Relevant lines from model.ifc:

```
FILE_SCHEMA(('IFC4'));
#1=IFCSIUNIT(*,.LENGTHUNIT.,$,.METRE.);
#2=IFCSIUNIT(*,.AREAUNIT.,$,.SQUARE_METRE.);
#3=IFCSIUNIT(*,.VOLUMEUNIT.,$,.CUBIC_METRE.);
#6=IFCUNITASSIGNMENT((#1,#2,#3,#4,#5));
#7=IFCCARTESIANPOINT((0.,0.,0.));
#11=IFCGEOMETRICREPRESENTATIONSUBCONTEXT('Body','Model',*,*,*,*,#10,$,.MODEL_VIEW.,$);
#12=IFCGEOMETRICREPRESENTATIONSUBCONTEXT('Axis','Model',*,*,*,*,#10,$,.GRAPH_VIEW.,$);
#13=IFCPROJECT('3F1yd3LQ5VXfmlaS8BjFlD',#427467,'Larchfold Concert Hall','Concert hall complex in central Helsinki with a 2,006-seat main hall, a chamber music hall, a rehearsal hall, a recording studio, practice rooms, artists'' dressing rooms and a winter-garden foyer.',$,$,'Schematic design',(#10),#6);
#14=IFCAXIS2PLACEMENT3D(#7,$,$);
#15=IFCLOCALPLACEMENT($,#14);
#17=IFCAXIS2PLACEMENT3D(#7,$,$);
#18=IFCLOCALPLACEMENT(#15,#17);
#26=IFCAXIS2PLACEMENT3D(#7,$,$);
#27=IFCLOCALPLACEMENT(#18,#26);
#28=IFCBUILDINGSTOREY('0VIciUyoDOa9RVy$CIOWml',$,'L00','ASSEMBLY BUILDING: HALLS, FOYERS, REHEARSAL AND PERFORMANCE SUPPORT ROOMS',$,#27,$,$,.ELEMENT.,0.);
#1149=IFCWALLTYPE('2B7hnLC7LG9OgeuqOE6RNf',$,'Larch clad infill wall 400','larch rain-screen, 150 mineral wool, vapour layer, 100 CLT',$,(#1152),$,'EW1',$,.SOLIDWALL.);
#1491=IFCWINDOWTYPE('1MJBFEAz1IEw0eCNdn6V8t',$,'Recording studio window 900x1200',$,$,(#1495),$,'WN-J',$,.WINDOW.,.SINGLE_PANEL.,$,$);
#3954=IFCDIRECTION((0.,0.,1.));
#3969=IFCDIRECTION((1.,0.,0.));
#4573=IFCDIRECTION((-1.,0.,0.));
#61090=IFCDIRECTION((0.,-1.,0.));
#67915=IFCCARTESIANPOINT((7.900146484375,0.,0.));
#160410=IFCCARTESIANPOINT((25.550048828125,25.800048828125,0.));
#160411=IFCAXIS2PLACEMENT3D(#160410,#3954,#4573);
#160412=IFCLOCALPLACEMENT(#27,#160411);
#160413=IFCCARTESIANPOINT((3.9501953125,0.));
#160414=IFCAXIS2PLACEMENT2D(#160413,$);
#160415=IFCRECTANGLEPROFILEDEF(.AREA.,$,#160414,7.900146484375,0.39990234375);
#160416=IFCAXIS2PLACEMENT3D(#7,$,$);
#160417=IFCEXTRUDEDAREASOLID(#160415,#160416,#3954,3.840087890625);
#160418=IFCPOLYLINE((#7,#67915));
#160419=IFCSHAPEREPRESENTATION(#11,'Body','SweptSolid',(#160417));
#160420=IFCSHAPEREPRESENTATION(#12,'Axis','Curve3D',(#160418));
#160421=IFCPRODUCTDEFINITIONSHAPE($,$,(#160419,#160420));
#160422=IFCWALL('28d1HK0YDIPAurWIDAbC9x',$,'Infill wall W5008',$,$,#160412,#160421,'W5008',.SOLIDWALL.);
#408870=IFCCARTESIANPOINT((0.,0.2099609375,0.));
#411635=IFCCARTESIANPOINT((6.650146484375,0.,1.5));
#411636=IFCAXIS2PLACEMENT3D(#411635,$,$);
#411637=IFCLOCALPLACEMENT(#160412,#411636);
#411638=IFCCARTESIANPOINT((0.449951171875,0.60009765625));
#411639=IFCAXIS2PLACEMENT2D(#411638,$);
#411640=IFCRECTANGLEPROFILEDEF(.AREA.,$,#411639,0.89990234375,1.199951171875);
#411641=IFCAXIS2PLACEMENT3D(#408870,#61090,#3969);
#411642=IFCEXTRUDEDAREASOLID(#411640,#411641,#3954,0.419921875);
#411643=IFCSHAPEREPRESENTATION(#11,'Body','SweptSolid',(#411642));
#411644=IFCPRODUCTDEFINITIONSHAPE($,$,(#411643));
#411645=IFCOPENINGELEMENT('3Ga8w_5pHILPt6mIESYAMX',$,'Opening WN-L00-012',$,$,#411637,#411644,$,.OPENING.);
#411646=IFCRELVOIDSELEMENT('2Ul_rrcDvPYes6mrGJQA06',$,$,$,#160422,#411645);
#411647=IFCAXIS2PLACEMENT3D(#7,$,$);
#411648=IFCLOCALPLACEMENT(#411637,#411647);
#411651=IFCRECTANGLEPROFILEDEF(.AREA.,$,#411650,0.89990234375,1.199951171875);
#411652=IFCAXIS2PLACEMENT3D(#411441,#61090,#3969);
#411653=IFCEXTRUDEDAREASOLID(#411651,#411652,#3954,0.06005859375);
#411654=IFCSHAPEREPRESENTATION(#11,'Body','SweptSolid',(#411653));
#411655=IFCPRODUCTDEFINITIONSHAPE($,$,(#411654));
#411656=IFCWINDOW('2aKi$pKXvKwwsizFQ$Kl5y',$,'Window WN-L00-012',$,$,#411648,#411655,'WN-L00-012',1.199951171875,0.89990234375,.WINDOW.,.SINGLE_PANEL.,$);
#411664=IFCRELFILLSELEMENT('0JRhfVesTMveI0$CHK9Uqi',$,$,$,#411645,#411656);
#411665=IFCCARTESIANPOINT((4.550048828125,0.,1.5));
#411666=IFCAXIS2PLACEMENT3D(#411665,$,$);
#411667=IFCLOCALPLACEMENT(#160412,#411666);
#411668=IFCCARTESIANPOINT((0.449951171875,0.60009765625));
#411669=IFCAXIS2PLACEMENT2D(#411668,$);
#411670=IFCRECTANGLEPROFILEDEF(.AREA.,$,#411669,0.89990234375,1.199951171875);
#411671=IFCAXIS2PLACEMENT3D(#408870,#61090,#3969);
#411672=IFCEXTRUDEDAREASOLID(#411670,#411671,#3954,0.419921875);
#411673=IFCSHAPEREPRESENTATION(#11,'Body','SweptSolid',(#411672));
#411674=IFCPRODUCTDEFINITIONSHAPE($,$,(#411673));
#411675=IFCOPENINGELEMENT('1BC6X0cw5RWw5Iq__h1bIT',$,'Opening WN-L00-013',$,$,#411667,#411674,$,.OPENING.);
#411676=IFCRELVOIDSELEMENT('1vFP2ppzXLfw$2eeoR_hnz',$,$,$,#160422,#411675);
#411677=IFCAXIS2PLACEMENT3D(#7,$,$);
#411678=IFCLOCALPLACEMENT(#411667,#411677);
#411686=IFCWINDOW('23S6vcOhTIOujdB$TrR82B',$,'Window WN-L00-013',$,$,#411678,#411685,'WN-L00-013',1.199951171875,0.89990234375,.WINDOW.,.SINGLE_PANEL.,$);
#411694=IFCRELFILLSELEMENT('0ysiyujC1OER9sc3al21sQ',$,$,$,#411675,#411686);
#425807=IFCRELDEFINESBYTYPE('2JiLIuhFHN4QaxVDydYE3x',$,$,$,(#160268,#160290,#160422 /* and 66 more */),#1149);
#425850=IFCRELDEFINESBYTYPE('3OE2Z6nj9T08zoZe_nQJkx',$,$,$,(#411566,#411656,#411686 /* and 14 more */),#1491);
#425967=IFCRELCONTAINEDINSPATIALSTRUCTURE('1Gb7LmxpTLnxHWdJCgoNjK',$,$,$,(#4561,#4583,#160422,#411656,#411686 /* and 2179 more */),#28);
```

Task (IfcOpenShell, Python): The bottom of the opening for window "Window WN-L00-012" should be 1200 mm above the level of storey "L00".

```python
import numpy as np
import ifcopenshell
import ifcopenshell.api.geometry
import ifcopenshell.geom
import ifcopenshell.util.element
import ifcopenshell.util.placement
import ifcopenshell.util.shape
import ifcopenshell.util.unit

model = ifcopenshell.open("model.ifc")
unit_scale = ifcopenshell.util.unit.calculate_unit_scale(model)

window = model.by_guid("2aKi$pKXvKwwsizFQ$Kl5y")
opening = window.FillsVoids[0].RelatingOpeningElement
storey = ifcopenshell.util.element.get_container(window, ifc_class="IfcBuildingStorey")
level = ifcopenshell.util.placement.get_local_placement(storey.ObjectPlacement)[2, 3]

# The opening's origin need not be at the sill, so measure its lowest point.
shape = ifcopenshell.geom.create_shape(ifcopenshell.geom.settings(), opening)
bottom = ifcopenshell.util.shape.get_shape_bottom_elevation(shape, shape.geometry) / unit_scale
dz = level + 1.2 - bottom

shift = np.array([0.0, 0.0, dz])
# The window is placed relative to its opening, so it follows when the opening moves.
matrix = ifcopenshell.util.placement.get_local_placement(opening.ObjectPlacement)
matrix[:3, 3] += shift
ifcopenshell.api.geometry.edit_object_placement(
    model, product=opening, matrix=matrix, is_si=False, should_transform_children=True
)

print(f"moved by {dz * unit_scale:+.3f} m")

model.write("model-out.ifc")
```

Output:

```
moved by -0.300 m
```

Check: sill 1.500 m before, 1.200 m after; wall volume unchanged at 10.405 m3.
